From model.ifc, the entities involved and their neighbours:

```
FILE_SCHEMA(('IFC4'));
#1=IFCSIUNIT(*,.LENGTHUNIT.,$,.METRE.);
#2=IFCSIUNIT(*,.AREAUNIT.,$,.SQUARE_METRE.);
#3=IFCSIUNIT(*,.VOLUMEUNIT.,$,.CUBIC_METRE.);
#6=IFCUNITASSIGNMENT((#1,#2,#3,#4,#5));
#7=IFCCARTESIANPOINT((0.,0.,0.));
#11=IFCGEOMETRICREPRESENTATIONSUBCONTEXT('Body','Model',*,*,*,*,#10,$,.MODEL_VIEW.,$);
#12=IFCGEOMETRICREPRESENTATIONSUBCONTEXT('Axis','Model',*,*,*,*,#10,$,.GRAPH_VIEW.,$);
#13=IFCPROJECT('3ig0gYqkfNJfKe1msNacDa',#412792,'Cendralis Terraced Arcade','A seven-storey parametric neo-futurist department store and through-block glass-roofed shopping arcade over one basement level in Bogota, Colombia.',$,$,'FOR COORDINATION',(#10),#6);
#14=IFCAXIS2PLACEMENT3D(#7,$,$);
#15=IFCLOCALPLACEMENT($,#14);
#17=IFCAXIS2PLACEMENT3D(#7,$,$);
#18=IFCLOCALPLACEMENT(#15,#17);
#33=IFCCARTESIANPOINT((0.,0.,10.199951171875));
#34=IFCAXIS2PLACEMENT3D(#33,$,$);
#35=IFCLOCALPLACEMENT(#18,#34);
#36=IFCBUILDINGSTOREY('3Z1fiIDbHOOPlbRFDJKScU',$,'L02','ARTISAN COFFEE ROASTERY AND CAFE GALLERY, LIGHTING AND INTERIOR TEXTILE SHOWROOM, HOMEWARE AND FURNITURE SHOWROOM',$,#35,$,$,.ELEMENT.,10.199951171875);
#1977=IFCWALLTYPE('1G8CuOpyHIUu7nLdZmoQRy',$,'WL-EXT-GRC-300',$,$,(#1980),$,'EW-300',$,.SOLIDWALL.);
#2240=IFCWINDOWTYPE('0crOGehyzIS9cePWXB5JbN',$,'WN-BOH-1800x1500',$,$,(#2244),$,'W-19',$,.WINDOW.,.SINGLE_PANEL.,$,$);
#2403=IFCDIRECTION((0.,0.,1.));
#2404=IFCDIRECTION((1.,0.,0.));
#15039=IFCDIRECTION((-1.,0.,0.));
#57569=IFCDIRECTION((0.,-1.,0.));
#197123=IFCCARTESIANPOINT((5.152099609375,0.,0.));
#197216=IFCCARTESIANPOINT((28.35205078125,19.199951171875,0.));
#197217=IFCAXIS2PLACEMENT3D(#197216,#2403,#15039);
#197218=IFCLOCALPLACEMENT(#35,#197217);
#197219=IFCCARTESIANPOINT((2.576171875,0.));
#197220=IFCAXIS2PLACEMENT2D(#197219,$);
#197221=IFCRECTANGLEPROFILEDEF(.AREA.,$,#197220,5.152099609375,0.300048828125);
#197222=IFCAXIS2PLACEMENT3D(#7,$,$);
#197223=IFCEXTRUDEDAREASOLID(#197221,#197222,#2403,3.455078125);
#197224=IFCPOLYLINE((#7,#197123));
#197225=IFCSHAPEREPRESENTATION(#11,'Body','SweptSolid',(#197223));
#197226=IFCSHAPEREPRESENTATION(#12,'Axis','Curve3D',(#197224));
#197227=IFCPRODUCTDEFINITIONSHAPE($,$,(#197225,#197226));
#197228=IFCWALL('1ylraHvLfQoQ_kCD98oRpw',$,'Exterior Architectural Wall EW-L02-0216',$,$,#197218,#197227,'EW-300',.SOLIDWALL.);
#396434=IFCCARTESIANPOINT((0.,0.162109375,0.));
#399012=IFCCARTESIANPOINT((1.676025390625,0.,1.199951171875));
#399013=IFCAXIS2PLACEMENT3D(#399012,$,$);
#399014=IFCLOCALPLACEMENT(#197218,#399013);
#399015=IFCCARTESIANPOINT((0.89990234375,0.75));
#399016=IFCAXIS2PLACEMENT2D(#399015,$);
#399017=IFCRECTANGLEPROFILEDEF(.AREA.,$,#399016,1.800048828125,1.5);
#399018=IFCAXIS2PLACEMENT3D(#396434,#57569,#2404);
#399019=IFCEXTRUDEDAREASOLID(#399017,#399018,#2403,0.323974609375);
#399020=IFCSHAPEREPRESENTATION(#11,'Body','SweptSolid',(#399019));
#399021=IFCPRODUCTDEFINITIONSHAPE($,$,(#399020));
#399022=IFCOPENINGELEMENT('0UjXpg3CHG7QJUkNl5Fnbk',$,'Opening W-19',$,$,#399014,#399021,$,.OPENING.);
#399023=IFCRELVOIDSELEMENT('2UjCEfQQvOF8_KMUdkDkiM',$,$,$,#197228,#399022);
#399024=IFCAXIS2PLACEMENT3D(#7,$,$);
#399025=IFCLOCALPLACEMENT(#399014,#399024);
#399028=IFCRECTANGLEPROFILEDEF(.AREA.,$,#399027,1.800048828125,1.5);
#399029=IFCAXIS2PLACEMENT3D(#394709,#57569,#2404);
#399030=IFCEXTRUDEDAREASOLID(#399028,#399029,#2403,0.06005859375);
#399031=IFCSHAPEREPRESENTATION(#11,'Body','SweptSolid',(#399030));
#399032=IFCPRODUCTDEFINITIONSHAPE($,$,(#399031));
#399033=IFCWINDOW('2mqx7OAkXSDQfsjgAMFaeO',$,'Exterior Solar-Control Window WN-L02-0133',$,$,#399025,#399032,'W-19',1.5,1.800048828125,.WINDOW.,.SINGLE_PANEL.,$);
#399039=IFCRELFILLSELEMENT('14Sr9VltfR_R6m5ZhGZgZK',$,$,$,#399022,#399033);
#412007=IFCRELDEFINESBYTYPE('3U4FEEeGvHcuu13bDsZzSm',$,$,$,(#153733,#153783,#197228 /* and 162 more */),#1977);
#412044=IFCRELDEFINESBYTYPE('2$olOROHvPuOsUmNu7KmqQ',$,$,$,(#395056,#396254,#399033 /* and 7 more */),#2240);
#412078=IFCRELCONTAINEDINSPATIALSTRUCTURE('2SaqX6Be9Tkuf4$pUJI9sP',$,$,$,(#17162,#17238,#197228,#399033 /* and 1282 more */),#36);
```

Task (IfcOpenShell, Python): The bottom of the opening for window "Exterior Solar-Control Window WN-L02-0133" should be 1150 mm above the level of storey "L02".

```python
import numpy as np
import ifcopenshell
import ifcopenshell.api.geometry
import ifcopenshell.geom
import ifcopenshell.util.element
import ifcopenshell.util.placement
import ifcopenshell.util.shape
import ifcopenshell.util.unit

model = ifcopenshell.open("model.ifc")
unit_scale = ifcopenshell.util.unit.calculate_unit_scale(model)

window = model.by_guid("2mqx7OAkXSDQfsjgAMFaeO")
opening = window.FillsVoids[0].RelatingOpeningElement
storey = ifcopenshell.util.element.get_container(window, ifc_class="IfcBuildingStorey")
level = ifcopenshell.util.placement.get_local_placement(storey.ObjectPlacement)[2, 3]

# The opening's origin need not be at the sill, so measure its lowest point.
shape = ifcopenshell.geom.create_shape(ifcopenshell.geom.settings(), opening)
bottom = ifcopenshell.util.shape.get_shape_bottom_elevation(shape, shape.geometry) / unit_scale
dz = level + 1.15 - bottom

shift = np.array([0.0, 0.0, dz])
# The window is placed relative to its opening, so it follows when the opening moves.
matrix = ifcopenshell.util.placement.get_local_placement(opening.ObjectPlacement)
matrix[:3, 3] += shift
ifcopenshell.api.geometry.edit_object_placement(
    model, product=opening, matrix=matrix, is_si=False, should_transform_children=True
)

print(f"moved by {dz * unit_scale:+.3f} m")

model.write("model_v2.ifc")
```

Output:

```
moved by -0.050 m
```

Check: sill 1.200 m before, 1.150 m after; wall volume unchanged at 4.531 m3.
